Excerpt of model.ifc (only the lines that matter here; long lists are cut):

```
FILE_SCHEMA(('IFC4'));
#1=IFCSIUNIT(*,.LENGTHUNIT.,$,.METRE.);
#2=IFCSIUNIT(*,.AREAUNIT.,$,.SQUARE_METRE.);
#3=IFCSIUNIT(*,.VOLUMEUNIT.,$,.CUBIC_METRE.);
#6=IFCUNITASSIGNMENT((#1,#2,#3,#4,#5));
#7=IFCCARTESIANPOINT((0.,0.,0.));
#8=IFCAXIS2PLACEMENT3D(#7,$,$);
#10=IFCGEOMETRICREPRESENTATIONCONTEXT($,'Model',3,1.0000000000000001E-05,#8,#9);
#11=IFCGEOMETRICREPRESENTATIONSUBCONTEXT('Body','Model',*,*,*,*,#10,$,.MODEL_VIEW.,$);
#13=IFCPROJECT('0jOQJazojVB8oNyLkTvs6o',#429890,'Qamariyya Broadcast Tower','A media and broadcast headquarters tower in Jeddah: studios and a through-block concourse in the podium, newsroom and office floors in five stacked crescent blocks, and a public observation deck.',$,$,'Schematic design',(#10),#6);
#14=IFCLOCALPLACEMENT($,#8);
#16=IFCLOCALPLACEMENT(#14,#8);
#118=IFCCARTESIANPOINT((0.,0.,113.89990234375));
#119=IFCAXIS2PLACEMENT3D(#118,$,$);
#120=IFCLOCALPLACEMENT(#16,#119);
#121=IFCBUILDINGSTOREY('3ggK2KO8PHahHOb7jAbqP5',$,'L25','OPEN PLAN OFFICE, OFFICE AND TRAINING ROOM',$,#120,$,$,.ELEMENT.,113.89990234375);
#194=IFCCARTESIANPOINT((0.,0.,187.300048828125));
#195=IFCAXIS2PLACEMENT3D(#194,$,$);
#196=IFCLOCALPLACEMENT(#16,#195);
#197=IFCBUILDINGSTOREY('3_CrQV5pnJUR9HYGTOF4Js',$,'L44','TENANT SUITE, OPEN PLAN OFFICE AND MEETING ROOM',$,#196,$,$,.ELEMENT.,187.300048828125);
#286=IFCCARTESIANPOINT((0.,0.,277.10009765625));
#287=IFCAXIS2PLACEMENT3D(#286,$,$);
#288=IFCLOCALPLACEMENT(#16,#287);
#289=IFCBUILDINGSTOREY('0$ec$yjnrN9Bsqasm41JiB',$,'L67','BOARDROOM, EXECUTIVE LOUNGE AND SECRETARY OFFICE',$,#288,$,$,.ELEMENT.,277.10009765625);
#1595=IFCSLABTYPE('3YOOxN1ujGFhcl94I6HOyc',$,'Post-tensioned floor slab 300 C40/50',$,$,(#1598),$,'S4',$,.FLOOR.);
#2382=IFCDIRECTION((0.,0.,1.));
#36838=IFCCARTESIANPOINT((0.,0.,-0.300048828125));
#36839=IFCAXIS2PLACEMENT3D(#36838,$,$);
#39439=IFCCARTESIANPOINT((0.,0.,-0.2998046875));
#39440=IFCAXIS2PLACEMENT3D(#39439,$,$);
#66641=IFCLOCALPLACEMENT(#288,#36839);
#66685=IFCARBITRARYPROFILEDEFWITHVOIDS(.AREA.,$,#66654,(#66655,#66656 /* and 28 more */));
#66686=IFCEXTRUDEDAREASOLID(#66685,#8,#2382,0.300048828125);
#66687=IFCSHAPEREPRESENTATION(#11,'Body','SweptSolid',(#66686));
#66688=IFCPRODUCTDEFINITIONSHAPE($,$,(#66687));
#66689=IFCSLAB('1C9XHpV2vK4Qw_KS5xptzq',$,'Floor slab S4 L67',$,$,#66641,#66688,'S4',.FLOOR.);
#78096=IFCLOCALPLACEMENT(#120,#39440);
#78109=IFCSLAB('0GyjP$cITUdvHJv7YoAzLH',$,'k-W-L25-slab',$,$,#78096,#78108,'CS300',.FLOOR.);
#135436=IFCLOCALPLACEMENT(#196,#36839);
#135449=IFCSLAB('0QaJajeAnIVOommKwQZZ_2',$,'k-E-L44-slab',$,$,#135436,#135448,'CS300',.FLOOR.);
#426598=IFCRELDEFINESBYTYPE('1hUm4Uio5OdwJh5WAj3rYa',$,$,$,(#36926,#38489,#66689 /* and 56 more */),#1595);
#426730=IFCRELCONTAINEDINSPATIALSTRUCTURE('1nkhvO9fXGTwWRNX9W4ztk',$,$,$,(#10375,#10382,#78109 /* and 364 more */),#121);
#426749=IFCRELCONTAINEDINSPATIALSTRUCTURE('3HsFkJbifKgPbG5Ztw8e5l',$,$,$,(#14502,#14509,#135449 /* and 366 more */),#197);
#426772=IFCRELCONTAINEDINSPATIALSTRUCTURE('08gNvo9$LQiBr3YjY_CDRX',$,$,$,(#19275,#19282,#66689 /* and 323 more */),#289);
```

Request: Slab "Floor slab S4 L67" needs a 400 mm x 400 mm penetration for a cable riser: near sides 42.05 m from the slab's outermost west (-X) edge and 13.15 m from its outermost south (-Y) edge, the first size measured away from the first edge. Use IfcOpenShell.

```python
import numpy as np
import ifcopenshell
import ifcopenshell.api.feature
import ifcopenshell.api.geometry
import ifcopenshell.api.root
import ifcopenshell.geom
import ifcopenshell.util.placement
import ifcopenshell.util.representation
import ifcopenshell.util.shape
import ifcopenshell.util.unit

model = ifcopenshell.open("model.ifc")
unit_scale = ifcopenshell.util.unit.calculate_unit_scale(model)
settings = ifcopenshell.geom.settings()


def volume(element):
    """Net volume in cubic metres, openings subtracted."""
    shape = ifcopenshell.geom.create_shape(settings, element)
    return ifcopenshell.util.shape.get_volume(shape.geometry)


slab = model.by_guid("1C9XHpV2vK4Qw_KS5xptzq")
before = volume(slab)

# Extent in the slab's own axes, in metres. The edges named are its -X and -Y sides.
slab_shape = ifcopenshell.geom.create_shape(settings, slab)
vertices = ifcopenshell.util.shape.get_vertices(slab_shape.geometry)
x_min, y_min, bottom = vertices.min(axis=0)
top = vertices[:, 2].max()

opening = ifcopenshell.api.root.create_entity(model, ifc_class="IfcOpeningElement", name="Cable riser opening", predefined_type="OPENING")
context = ifcopenshell.util.representation.get_context(model, "Model", "Body", "MODEL_VIEW")
width, depth = 0.4, 0.4
outline = [(0.0, 0.0), (width, 0.0), (width, depth), (0.0, depth), (0.0, 0.0)]
# Overshoot both faces by 50 mm so the cut is clean.
shape = ifcopenshell.api.geometry.add_slab_representation(
    model, context=context, depth=top - bottom + 0.1, polyline=outline
)
ifcopenshell.api.geometry.assign_representation(model, product=opening, representation=shape)

matrix = ifcopenshell.util.placement.get_local_placement(slab.ObjectPlacement)
matrix[:, 3] = matrix @ np.append(np.array([x_min + 42.05, y_min + 13.15, bottom - 0.05]) / unit_scale, 1.0)
ifcopenshell.api.geometry.edit_object_placement(model, product=opening, matrix=matrix, is_si=False)
ifcopenshell.api.feature.add_feature(model, feature=opening, element=slab)

after = volume(slab)

print(f"slab volume {before:.3f} -> {after:.3f} m3")

model.write("model_rev.ifc")
```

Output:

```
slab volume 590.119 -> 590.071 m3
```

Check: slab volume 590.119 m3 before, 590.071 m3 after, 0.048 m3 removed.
